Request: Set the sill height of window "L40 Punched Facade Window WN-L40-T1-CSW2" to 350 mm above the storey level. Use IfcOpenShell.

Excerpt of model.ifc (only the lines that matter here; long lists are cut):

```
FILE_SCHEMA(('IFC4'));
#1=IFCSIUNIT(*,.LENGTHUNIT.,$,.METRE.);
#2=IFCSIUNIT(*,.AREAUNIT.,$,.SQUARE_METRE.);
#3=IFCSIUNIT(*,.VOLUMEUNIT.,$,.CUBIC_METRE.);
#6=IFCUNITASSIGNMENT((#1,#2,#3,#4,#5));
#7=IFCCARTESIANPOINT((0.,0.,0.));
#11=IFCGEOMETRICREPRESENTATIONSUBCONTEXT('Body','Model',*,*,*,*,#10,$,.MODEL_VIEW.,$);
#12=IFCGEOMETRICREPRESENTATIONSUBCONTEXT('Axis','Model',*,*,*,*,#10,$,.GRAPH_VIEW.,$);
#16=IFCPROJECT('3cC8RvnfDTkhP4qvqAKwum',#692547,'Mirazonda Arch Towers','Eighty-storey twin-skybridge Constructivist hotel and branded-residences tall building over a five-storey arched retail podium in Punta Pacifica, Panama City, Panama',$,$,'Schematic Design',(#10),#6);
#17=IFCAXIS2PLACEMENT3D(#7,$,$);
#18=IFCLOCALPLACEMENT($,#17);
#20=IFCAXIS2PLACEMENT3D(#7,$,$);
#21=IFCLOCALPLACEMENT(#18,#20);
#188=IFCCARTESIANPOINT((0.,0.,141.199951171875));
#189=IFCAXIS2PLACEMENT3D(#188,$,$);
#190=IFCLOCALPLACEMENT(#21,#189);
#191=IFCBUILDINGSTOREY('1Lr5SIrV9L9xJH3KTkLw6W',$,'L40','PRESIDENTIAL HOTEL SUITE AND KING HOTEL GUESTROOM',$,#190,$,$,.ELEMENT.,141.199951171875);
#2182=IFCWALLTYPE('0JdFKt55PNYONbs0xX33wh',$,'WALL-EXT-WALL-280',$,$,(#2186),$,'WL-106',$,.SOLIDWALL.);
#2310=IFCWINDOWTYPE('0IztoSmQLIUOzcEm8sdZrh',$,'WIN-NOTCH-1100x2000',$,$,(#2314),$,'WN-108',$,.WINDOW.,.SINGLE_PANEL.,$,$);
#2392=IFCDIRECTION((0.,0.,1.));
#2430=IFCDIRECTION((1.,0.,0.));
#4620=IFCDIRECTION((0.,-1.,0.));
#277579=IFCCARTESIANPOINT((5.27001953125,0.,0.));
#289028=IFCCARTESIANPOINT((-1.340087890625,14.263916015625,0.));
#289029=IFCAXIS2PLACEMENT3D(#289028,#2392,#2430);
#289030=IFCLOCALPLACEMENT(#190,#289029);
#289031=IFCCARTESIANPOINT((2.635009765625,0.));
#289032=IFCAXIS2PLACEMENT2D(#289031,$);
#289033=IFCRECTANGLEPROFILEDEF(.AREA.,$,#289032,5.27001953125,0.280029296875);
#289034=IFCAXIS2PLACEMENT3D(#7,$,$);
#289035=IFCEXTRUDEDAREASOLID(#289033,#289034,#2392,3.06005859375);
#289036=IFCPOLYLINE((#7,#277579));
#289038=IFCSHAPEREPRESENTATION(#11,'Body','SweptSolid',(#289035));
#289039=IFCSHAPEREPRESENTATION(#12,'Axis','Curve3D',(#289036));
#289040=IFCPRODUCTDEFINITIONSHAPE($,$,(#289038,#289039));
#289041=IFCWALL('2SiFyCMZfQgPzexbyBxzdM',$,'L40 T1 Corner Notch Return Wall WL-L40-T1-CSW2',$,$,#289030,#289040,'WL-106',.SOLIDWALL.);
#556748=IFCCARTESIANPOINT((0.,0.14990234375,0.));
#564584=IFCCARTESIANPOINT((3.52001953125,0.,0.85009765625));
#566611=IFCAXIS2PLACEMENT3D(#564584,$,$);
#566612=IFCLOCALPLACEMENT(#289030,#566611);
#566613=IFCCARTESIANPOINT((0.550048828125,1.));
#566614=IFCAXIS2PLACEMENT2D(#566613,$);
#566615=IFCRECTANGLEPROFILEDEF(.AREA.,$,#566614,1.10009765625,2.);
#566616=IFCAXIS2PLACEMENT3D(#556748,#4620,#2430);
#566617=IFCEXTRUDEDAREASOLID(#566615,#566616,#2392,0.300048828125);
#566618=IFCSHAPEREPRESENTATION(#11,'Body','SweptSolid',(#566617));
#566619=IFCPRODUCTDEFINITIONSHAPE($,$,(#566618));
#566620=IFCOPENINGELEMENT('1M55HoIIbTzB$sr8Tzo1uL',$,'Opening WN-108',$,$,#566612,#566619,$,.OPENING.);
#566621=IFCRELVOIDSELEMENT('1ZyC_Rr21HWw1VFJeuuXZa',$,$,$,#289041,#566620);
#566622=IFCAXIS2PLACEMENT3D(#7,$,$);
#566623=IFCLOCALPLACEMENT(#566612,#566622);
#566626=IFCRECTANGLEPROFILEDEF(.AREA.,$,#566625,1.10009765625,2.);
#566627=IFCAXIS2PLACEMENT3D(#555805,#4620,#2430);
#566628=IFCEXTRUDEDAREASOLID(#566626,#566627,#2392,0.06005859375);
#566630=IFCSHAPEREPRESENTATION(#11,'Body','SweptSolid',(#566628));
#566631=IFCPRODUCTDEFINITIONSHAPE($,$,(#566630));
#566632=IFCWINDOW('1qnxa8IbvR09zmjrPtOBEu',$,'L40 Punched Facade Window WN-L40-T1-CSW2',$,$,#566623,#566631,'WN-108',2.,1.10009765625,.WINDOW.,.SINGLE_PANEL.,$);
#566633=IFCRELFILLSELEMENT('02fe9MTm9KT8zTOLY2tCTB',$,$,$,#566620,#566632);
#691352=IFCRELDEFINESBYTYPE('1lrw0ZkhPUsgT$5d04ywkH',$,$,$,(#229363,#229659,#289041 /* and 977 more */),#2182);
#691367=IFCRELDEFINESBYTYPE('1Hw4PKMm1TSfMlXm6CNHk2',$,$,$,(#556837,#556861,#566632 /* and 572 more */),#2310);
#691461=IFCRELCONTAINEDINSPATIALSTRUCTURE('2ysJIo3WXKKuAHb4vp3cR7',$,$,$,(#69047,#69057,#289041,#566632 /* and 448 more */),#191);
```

```python
import numpy as np
import ifcopenshell
import ifcopenshell.api.geometry
import ifcopenshell.geom
import ifcopenshell.util.element
import ifcopenshell.util.placement
import ifcopenshell.util.shape
import ifcopenshell.util.unit

model = ifcopenshell.open("model.ifc")
unit_scale = ifcopenshell.util.unit.calculate_unit_scale(model)

window = model.by_guid("1qnxa8IbvR09zmjrPtOBEu")
opening = window.FillsVoids[0].RelatingOpeningElement
storey = ifcopenshell.util.element.get_container(window, ifc_class="IfcBuildingStorey")
level = ifcopenshell.util.placement.get_local_placement(storey.ObjectPlacement)[2, 3]

# The opening's origin need not be at the sill, so measure its lowest point.
shape = ifcopenshell.geom.create_shape(ifcopenshell.geom.settings(), opening)
bottom = ifcopenshell.util.shape.get_shape_bottom_elevation(shape, shape.geometry) / unit_scale
dz = level + 0.35 - bottom

shift = np.array([0.0, 0.0, dz])
# The window is placed relative to its opening, so it follows when the opening moves.
matrix = ifcopenshell.util.placement.get_local_placement(opening.ObjectPlacement)
matrix[:3, 3] += shift
ifcopenshell.api.geometry.edit_object_placement(
    model, product=opening, matrix=matrix, is_si=False, should_transform_children=True
)

print(f"moved by {dz * unit_scale:+.3f} m")

model.write("model_v2.ifc")
```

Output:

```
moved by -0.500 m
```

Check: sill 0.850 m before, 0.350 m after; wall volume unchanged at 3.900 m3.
